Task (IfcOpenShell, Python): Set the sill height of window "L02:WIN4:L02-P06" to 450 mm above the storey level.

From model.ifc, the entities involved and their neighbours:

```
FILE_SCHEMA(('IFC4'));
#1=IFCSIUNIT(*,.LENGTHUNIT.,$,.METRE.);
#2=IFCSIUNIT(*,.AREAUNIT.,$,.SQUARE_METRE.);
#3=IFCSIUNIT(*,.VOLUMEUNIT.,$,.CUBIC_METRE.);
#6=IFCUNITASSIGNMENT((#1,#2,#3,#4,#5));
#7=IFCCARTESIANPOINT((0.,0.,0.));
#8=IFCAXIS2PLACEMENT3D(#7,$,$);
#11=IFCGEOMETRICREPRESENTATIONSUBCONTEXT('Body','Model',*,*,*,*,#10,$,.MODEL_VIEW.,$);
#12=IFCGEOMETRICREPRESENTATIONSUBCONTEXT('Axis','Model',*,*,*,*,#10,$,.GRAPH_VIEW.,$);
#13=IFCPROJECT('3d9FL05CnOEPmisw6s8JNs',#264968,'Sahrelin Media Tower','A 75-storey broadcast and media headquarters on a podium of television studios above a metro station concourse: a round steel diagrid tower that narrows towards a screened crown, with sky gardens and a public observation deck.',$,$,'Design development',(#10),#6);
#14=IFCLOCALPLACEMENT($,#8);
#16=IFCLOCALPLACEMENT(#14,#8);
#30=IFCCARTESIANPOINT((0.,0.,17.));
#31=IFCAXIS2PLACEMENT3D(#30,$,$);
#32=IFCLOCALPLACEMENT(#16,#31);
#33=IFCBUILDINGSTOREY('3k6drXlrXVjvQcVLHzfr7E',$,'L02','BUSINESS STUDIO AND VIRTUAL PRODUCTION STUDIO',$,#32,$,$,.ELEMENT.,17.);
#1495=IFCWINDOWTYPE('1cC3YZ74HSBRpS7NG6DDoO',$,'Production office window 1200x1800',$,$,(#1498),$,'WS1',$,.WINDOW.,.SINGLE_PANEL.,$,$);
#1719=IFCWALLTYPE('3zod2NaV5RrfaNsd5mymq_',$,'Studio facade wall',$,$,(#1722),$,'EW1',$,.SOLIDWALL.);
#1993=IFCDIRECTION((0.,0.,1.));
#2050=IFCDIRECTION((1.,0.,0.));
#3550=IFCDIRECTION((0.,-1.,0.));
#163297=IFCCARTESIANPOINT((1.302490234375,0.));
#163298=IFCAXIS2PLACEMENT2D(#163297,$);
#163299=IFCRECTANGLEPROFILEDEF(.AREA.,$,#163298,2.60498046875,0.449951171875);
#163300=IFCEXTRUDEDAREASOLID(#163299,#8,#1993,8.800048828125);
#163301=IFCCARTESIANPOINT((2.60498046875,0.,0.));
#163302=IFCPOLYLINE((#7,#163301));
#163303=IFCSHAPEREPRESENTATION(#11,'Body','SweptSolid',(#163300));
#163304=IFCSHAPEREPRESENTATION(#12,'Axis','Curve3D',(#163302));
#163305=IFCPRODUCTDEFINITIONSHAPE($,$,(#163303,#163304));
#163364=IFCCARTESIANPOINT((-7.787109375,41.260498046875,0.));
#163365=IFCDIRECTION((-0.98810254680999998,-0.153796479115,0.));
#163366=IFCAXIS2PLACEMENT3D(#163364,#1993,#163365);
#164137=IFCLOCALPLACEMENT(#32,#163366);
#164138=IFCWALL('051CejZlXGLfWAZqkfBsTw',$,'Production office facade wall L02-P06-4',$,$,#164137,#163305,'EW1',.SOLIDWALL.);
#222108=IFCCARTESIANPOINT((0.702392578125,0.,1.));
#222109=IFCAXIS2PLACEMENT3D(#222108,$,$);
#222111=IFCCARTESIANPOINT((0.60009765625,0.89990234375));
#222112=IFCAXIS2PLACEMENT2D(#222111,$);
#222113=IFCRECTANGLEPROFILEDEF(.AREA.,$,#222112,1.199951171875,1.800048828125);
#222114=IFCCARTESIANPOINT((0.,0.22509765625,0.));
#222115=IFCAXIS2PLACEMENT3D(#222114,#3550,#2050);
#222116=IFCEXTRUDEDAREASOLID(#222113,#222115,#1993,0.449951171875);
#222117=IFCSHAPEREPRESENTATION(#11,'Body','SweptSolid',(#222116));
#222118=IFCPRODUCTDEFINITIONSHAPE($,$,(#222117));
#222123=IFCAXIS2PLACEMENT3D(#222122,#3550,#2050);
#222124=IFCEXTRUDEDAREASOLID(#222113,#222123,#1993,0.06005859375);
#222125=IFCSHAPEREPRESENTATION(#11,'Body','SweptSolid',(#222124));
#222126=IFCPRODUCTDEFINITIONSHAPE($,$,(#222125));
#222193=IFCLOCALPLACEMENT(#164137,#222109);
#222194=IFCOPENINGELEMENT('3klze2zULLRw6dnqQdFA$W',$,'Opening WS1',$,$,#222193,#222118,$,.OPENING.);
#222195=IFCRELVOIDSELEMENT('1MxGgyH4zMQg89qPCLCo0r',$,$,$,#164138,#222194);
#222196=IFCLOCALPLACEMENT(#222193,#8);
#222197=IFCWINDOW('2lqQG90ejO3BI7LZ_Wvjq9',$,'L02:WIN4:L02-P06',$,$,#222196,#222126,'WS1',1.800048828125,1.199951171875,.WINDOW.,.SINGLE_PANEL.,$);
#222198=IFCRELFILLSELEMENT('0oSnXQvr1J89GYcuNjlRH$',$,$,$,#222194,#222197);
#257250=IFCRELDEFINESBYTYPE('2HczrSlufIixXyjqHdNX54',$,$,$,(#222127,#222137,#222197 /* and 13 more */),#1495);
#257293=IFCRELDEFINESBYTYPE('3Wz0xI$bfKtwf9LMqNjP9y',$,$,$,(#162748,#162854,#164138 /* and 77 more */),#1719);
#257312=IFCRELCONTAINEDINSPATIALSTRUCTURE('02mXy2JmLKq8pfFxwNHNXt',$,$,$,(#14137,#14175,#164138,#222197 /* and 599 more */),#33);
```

```python
import numpy as np
import ifcopenshell
import ifcopenshell.api.geometry
import ifcopenshell.geom
import ifcopenshell.util.element
import ifcopenshell.util.placement
import ifcopenshell.util.shape
import ifcopenshell.util.unit

model = ifcopenshell.open("model.ifc")
unit_scale = ifcopenshell.util.unit.calculate_unit_scale(model)

window = model.by_id(222197)
opening = window.FillsVoids[0].RelatingOpeningElement
storey = ifcopenshell.util.element.get_container(window, ifc_class="IfcBuildingStorey")
level = ifcopenshell.util.placement.get_local_placement(storey.ObjectPlacement)[2, 3]

# The opening's origin need not be at the sill, so measure its lowest point.
shape = ifcopenshell.geom.create_shape(ifcopenshell.geom.settings(), opening)
bottom = ifcopenshell.util.shape.get_shape_bottom_elevation(shape, shape.geometry) / unit_scale
dz = level + 0.45 - bottom

shift = np.array([0.0, 0.0, dz])
# The window is placed relative to its opening, so it follows when the opening moves.
matrix = ifcopenshell.util.placement.get_local_placement(opening.ObjectPlacement)
matrix[:3, 3] += shift
ifcopenshell.api.geometry.edit_object_placement(
    model, product=opening, matrix=matrix, is_si=False, should_transform_children=True
)

print(f"moved by {dz * unit_scale:+.3f} m")

model.write("model_edited.ifc")
```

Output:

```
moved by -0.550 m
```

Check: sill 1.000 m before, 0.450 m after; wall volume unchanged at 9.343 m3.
